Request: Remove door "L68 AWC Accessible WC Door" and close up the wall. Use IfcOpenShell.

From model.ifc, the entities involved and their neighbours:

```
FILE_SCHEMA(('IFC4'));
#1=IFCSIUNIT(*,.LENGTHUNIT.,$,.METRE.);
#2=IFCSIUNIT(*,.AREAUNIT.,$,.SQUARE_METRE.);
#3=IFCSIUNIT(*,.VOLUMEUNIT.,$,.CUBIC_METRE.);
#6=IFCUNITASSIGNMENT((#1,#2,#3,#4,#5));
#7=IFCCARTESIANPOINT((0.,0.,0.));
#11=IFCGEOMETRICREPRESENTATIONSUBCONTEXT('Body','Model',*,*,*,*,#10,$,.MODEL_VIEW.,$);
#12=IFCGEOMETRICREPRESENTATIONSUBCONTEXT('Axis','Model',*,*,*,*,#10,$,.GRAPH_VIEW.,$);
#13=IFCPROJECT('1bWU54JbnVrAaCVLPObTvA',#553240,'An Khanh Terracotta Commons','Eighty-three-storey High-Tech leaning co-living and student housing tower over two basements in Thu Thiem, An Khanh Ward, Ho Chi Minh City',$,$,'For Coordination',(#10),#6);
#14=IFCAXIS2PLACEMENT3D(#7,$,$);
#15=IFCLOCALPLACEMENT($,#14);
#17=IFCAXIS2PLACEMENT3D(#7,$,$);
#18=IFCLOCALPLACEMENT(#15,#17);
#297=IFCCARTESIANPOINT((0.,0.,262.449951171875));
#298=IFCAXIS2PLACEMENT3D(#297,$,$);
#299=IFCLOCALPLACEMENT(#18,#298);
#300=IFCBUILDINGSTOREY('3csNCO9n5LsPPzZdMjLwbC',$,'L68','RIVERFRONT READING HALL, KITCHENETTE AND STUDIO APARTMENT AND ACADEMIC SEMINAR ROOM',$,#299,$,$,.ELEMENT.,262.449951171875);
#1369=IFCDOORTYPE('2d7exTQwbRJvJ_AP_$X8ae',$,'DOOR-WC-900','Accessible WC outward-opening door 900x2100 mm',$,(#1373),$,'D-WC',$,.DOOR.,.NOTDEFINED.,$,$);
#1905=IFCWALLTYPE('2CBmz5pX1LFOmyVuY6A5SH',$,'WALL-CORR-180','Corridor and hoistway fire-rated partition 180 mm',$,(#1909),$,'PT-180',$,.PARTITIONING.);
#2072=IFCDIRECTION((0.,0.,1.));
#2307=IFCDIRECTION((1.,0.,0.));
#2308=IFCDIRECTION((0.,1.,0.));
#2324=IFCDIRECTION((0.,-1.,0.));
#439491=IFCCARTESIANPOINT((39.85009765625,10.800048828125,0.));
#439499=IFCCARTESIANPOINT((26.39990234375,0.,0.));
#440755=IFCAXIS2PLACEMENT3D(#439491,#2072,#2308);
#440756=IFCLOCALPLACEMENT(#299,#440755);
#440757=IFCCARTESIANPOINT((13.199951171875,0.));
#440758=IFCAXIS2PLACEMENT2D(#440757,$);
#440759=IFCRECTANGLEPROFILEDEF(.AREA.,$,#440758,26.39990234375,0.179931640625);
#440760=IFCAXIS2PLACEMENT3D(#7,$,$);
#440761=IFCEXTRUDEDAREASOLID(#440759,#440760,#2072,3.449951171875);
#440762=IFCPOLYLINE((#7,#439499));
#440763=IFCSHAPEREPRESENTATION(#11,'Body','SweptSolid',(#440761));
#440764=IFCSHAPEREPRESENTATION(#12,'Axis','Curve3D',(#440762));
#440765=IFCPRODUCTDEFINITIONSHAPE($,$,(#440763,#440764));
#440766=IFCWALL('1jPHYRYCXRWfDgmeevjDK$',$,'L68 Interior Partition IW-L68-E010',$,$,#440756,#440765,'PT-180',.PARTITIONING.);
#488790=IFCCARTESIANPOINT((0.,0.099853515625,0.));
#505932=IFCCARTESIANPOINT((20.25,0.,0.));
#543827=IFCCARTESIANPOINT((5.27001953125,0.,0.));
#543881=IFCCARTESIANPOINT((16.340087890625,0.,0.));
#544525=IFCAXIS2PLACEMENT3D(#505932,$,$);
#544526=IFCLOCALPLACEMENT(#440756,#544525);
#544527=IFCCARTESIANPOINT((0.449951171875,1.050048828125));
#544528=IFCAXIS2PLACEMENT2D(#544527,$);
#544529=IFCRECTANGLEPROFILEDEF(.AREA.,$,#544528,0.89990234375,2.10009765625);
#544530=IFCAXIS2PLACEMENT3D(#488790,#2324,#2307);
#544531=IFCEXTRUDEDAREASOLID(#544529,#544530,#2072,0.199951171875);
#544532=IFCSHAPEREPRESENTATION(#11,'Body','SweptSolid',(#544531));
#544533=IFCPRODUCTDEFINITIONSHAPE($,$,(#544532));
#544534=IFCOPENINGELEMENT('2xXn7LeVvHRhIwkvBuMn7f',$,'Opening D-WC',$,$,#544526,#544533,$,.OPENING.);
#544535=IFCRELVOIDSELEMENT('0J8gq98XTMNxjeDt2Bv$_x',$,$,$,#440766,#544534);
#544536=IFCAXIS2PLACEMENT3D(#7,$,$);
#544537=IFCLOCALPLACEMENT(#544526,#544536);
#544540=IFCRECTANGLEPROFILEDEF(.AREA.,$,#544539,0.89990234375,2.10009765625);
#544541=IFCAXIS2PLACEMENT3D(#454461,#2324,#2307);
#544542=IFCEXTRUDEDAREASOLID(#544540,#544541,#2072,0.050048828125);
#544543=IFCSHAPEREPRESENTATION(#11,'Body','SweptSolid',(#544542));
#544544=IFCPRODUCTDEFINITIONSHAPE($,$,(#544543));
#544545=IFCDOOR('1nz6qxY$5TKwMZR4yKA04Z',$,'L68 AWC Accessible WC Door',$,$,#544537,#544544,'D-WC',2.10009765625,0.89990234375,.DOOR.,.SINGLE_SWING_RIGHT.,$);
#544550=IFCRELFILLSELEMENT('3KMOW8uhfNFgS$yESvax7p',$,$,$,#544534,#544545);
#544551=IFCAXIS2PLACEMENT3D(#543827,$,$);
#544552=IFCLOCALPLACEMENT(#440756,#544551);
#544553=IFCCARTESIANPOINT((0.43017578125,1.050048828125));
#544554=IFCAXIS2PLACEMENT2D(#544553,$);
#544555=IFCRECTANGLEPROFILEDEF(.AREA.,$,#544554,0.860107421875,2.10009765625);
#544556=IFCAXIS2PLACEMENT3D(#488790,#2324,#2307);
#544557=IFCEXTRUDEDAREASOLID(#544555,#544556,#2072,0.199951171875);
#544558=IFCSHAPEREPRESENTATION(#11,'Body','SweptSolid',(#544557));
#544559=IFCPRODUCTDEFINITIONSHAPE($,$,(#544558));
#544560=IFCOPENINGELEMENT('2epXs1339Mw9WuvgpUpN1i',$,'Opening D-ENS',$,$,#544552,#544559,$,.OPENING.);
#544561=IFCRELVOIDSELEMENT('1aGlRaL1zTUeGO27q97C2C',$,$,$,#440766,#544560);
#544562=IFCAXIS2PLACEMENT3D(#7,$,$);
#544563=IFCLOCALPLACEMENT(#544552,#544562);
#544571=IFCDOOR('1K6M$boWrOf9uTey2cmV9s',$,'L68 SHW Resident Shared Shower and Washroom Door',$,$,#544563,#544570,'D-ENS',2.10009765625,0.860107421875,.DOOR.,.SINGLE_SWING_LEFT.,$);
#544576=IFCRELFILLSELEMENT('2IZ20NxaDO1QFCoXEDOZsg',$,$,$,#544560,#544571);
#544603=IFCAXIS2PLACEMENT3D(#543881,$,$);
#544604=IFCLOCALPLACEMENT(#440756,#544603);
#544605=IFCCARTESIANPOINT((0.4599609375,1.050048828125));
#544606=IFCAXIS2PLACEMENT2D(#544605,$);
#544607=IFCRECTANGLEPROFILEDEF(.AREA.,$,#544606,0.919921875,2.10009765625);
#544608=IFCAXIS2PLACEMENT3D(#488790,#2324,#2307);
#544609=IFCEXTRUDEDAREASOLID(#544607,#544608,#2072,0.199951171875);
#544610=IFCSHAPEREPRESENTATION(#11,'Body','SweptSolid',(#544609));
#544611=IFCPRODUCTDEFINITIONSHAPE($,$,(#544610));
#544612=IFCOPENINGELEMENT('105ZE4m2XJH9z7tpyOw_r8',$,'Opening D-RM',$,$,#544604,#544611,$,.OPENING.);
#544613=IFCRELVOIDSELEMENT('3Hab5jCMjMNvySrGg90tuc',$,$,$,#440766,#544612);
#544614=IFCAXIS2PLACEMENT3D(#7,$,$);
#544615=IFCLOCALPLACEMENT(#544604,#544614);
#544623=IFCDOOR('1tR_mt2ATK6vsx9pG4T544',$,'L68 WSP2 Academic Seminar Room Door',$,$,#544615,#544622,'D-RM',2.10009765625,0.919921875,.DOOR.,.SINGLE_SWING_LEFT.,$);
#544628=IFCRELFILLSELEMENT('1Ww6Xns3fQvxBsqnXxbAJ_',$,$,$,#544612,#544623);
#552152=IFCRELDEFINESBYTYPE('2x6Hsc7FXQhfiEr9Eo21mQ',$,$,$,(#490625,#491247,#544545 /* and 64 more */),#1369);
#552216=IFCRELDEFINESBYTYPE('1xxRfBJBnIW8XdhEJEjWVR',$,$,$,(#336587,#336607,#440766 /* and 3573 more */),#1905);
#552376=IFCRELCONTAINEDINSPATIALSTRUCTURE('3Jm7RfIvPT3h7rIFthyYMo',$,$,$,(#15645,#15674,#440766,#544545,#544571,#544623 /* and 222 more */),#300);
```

```python
import ifcopenshell
import ifcopenshell.api.feature
import ifcopenshell.api.root
import ifcopenshell.geom
import ifcopenshell.util.shape

model = ifcopenshell.open("model.ifc")
settings = ifcopenshell.geom.settings()


def volume(element):
    """Net volume in cubic metres, openings subtracted."""
    shape = ifcopenshell.geom.create_shape(settings, element)
    return ifcopenshell.util.shape.get_volume(shape.geometry)


door = model.by_guid("1nz6qxY$5TKwMZR4yKA04Z")
opening = door.FillsVoids[0].RelatingOpeningElement
wall = opening.VoidsElements[0].RelatingBuildingElement
before = volume(wall)

ifcopenshell.api.root.remove_product(model, product=door)
ifcopenshell.api.feature.remove_feature(model, feature=opening)

after = volume(wall)

print(f"wall volume {before:.3f} -> {after:.3f} m3")

model.write("model_edited.ifc")
```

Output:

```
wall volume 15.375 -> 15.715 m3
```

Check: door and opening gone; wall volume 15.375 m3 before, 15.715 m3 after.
